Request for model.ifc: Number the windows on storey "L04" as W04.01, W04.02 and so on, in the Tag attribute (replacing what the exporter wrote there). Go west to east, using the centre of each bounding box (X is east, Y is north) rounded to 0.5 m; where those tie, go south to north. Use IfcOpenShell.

First a look at what the model holds.

```python
import ifcopenshell
import ifcopenshell.util.element
import ifcopenshell.util.placement

model = ifcopenshell.open("model.ifc")
print(model.schema)
storey = next(s for s in model.by_type("IfcBuildingStorey") if s.Name == "L04")
windows = [e for e in ifcopenshell.util.element.get_decomposition(storey) if e.is_a("IfcWindow")]
for e in sorted(windows, key=lambda e: e.id()):
    origin = ifcopenshell.util.placement.get_local_placement(e.ObjectPlacement)[:3, 3]
    print(e.id(), e.Tag, e.Name, origin.round(2) + 0.0, sep=" | ")
```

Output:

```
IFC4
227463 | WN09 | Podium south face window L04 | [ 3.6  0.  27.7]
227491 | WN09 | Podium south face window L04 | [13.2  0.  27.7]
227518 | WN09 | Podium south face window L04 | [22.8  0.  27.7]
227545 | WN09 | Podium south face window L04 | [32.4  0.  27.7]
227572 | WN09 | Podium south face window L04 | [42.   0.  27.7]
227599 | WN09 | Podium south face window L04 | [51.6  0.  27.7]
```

```python
import ifcopenshell
import ifcopenshell.geom
import ifcopenshell.util.element
import ifcopenshell.util.shape

model = ifcopenshell.open("model.ifc")
settings = ifcopenshell.geom.settings()
settings.set("use-world-coords", True)


def centre(element):
    shape = ifcopenshell.geom.create_shape(settings, element)
    return ifcopenshell.util.shape.get_bbox_centroid(shape.geometry)


storey = next(s for s in model.by_type("IfcBuildingStorey") if s.Name == "L04")
windows = [e for e in ifcopenshell.util.element.get_decomposition(storey) if e.is_a("IfcWindow")]

# Insertion points can sit at a corner or the storey origin, so sort by the geometry (in metres).
centres = {e: centre(e) for e in windows}
windows.sort(key=lambda e: (round(centres[e][0] / 0.5), centres[e][1]))

for i, e in enumerate(windows, start=1):
    number = f"W04.{i:02d}"
    e.Tag = number
    print(e.id(), number)

model.write("model_edited.ifc")
```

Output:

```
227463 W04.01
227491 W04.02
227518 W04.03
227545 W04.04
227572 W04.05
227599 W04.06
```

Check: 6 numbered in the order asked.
